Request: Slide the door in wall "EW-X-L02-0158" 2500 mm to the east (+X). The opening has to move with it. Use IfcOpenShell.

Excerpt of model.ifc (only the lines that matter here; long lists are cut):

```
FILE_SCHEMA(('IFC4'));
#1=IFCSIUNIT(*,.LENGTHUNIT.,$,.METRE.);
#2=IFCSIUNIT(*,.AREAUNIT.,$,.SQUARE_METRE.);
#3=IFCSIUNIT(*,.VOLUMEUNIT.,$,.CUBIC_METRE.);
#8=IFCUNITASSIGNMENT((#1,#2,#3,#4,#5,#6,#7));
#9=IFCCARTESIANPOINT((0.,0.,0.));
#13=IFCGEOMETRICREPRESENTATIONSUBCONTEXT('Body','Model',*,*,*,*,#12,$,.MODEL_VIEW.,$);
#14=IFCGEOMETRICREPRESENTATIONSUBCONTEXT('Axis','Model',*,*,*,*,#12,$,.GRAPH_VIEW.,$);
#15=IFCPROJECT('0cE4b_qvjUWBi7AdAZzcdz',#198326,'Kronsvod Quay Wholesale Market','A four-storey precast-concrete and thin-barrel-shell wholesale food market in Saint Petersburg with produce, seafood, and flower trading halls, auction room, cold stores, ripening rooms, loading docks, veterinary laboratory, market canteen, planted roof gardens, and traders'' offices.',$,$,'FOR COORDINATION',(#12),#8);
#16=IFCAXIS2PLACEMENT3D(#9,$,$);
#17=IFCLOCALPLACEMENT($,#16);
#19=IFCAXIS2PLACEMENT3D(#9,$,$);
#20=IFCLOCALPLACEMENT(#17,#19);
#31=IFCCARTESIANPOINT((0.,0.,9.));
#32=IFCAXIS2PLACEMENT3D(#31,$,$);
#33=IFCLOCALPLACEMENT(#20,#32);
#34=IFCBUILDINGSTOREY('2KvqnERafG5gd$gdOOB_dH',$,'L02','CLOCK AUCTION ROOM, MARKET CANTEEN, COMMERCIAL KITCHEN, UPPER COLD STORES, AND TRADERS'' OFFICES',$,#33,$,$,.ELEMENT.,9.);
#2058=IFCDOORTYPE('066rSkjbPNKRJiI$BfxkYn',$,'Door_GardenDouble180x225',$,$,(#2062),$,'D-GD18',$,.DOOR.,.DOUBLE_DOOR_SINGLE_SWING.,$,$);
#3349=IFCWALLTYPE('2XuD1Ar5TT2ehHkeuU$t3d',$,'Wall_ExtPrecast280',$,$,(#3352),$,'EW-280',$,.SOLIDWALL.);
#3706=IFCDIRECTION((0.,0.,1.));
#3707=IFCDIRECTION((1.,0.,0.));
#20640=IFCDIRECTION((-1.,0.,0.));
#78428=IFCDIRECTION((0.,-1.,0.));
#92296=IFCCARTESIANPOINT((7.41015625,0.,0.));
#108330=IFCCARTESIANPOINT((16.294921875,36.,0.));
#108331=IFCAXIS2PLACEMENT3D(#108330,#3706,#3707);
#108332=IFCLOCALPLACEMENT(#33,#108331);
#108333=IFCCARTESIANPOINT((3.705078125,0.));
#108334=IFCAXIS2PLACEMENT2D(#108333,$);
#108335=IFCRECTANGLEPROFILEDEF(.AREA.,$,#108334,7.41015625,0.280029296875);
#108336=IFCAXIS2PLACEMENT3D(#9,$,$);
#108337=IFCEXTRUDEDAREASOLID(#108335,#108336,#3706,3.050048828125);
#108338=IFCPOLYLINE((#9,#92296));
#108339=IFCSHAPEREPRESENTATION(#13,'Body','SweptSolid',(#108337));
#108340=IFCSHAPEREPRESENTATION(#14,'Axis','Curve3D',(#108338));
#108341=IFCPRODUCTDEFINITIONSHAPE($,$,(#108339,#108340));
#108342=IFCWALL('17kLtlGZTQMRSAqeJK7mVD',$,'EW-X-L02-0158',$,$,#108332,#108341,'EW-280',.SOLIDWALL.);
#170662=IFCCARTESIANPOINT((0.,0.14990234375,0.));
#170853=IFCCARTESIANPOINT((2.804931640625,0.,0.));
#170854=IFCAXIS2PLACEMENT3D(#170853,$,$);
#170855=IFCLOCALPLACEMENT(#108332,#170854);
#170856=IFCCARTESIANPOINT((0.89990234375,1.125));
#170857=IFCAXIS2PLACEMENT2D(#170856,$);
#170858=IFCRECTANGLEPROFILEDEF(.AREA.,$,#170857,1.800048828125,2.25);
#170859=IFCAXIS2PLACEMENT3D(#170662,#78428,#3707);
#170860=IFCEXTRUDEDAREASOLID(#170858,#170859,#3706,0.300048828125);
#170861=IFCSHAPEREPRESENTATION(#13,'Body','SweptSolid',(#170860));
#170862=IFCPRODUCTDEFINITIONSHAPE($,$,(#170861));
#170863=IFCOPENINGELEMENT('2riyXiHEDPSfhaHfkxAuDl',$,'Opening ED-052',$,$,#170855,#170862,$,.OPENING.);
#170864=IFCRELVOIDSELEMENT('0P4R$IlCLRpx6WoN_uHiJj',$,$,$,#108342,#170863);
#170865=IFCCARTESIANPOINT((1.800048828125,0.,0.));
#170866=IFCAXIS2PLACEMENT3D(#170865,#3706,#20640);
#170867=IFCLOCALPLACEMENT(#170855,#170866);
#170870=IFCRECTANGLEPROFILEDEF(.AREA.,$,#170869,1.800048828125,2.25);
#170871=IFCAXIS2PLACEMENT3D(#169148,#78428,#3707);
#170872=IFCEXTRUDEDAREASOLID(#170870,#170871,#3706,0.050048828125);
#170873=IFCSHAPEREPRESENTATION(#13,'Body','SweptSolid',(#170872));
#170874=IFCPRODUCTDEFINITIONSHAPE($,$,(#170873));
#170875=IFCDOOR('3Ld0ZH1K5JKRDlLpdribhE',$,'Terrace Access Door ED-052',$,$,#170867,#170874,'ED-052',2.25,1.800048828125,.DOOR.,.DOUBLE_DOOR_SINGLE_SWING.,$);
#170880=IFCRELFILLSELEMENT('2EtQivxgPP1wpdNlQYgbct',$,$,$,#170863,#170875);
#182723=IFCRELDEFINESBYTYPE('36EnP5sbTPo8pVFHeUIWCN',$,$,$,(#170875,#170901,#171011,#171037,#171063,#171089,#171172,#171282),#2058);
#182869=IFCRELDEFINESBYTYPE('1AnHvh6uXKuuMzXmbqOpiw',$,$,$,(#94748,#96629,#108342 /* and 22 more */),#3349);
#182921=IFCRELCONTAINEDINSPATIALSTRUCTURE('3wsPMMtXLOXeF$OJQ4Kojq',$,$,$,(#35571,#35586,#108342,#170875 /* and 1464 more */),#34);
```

```python
import ifcopenshell
import ifcopenshell.api.geometry
import ifcopenshell.util.placement

model = ifcopenshell.open("model.ifc")

door = model.by_id(170875)
opening = door.FillsVoids[0].RelatingOpeningElement
wall = opening.VoidsElements[0].RelatingBuildingElement

wall_matrix = ifcopenshell.util.placement.get_local_placement(wall.ObjectPlacement)
shift = wall_matrix[:3, 0] * 2.5
before = ifcopenshell.util.placement.get_local_placement(door.ObjectPlacement)[:3, 3].copy()

# The door is placed relative to its opening, so it follows when the opening moves.
matrix = ifcopenshell.util.placement.get_local_placement(opening.ObjectPlacement)
matrix[:3, 3] += shift
ifcopenshell.api.geometry.edit_object_placement(
    model, product=opening, matrix=matrix, is_si=False, should_transform_children=True
)

after = ifcopenshell.util.placement.get_local_placement(door.ObjectPlacement)[:3, 3]
print("door moved by", (after - before).round(3) + 0.0)

model.write("model-out.ifc")
```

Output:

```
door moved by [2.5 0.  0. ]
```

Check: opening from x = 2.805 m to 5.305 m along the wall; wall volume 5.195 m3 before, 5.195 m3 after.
